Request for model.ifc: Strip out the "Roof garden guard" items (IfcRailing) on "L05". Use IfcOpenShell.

First a look at what the model holds.

```python
import ifcopenshell
import ifcopenshell.util.element

model = ifcopenshell.open("model.ifc")
print(model.schema)
storey = next(s for s in model.by_type("IfcBuildingStorey") if s.Name == "L05")
railings = [e for e in ifcopenshell.util.element.get_decomposition(storey) if e.is_a("IfcRailing")]
seen = {}
for e in railings:
    element_type = ifcopenshell.util.element.get_type(e)
    name = element_type.Name if element_type not in (None, e) else None
    seen[name] = seen.get(name, 0) + 1
for name, count in sorted(seen.items(), key=str):
    print(count, "x", name)
```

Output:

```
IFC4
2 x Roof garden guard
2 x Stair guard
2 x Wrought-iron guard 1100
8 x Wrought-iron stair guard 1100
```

```python
import ifcopenshell
import ifcopenshell.api.root
import ifcopenshell.util.element

model = ifcopenshell.open("model.ifc")

storey = next(s for s in model.by_type("IfcBuildingStorey") if s.Name == "L05")
railings = [e for e in ifcopenshell.util.element.get_decomposition(storey) if e.is_a("IfcRailing")]
targets = [e for e in railings if (t := ifcopenshell.util.element.get_type(e)) not in (None, e) and t.Name == "Roof garden guard"]

for e in targets:
    ifcopenshell.api.root.remove_product(model, product=e)
print(len(targets), "removed")

model.write("model_updated.ifc")
```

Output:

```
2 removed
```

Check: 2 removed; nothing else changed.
